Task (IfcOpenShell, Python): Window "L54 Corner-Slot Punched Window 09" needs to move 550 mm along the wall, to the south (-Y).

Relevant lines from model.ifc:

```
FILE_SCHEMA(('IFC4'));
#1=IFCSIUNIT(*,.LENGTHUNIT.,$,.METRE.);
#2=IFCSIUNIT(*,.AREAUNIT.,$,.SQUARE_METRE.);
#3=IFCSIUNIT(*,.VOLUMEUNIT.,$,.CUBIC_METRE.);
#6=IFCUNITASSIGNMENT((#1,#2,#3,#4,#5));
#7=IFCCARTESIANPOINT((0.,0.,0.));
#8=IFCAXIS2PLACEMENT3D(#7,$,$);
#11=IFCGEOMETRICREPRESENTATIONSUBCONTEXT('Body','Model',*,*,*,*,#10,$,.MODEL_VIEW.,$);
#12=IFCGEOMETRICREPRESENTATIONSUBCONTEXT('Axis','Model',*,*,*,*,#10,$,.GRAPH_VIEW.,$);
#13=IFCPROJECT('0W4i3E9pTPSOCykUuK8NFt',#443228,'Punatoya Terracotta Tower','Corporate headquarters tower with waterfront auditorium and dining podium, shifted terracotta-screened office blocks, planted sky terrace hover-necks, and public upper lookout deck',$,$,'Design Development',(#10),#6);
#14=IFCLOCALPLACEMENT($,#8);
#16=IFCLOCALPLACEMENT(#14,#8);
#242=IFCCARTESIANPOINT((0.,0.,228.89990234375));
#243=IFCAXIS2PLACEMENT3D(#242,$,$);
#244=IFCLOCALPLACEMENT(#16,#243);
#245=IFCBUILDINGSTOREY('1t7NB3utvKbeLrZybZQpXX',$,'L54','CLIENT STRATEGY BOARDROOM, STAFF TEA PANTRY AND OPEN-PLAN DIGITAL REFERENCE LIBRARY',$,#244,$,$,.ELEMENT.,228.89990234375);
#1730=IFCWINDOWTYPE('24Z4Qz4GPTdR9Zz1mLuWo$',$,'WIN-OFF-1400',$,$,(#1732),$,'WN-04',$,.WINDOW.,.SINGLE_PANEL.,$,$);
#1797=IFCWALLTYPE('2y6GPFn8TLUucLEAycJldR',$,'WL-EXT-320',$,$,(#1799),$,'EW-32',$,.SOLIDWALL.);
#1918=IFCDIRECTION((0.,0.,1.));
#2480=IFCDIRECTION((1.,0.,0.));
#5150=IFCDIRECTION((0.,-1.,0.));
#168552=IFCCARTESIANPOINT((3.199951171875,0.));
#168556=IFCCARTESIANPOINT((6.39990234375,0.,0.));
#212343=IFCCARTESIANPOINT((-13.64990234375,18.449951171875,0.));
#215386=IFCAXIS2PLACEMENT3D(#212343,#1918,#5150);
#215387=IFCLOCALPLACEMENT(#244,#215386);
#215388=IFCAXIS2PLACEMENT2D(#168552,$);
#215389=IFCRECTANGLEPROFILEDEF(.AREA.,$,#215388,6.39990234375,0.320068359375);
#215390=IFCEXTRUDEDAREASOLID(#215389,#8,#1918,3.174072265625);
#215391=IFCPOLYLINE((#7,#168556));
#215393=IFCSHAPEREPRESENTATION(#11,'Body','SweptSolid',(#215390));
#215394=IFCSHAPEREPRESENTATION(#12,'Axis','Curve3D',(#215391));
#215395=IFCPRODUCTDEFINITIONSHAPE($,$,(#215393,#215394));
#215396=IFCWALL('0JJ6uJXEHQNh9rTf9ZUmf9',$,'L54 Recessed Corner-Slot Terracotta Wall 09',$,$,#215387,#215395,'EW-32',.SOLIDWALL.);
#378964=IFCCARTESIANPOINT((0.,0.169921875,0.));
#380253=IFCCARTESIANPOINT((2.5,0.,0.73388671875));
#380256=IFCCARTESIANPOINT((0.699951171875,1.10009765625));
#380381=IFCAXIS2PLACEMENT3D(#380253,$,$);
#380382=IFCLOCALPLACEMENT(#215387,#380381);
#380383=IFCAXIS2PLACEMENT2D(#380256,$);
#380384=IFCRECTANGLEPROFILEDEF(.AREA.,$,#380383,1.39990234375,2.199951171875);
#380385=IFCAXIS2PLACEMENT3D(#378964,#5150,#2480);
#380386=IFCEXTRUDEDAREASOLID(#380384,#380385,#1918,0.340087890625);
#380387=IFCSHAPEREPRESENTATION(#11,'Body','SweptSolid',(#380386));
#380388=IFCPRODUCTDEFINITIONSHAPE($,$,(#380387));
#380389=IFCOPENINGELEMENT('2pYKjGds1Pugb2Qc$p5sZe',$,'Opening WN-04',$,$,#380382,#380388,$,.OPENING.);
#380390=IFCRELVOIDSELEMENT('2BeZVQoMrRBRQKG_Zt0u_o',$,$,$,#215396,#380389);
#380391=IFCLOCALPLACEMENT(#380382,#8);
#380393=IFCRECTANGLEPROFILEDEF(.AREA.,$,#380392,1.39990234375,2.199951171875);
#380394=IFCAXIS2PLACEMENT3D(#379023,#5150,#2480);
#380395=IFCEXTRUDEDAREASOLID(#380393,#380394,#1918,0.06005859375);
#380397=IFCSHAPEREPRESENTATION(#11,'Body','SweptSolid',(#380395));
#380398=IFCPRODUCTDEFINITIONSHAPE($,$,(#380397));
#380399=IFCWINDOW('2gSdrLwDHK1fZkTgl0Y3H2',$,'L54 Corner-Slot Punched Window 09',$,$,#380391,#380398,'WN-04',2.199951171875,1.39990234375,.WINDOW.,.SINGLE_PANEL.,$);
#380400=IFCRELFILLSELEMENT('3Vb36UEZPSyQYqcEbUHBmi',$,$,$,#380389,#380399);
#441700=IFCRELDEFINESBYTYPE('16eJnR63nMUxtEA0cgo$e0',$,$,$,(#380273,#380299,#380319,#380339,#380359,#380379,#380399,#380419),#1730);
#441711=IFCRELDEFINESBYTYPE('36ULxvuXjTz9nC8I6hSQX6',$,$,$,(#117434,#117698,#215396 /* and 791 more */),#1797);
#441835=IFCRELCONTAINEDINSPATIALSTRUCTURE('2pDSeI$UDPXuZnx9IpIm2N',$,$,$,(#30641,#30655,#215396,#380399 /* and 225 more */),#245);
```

```python
import ifcopenshell
import ifcopenshell.api.geometry
import ifcopenshell.util.placement
import ifcopenshell.util.unit

model = ifcopenshell.open("model.ifc")
unit_scale = ifcopenshell.util.unit.calculate_unit_scale(model)

window = model.by_guid("2gSdrLwDHK1fZkTgl0Y3H2")
opening = window.FillsVoids[0].RelatingOpeningElement
wall = opening.VoidsElements[0].RelatingBuildingElement

wall_matrix = ifcopenshell.util.placement.get_local_placement(wall.ObjectPlacement)
shift = wall_matrix[:3, 0] * 0.55 / unit_scale
before = ifcopenshell.util.placement.get_local_placement(window.ObjectPlacement)[:3, 3].copy()

# The window is placed relative to its opening, so it follows when the opening moves.
matrix = ifcopenshell.util.placement.get_local_placement(opening.ObjectPlacement)
matrix[:3, 3] += shift
ifcopenshell.api.geometry.edit_object_placement(
    model, product=opening, matrix=matrix, is_si=False, should_transform_children=True
)

after = ifcopenshell.util.placement.get_local_placement(window.ObjectPlacement)[:3, 3]
print("window moved by", (after - before).round(3) + 0.0)

model.write("model_v2.ifc")
```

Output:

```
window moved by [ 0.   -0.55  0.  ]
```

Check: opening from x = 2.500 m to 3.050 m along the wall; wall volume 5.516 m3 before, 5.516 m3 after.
